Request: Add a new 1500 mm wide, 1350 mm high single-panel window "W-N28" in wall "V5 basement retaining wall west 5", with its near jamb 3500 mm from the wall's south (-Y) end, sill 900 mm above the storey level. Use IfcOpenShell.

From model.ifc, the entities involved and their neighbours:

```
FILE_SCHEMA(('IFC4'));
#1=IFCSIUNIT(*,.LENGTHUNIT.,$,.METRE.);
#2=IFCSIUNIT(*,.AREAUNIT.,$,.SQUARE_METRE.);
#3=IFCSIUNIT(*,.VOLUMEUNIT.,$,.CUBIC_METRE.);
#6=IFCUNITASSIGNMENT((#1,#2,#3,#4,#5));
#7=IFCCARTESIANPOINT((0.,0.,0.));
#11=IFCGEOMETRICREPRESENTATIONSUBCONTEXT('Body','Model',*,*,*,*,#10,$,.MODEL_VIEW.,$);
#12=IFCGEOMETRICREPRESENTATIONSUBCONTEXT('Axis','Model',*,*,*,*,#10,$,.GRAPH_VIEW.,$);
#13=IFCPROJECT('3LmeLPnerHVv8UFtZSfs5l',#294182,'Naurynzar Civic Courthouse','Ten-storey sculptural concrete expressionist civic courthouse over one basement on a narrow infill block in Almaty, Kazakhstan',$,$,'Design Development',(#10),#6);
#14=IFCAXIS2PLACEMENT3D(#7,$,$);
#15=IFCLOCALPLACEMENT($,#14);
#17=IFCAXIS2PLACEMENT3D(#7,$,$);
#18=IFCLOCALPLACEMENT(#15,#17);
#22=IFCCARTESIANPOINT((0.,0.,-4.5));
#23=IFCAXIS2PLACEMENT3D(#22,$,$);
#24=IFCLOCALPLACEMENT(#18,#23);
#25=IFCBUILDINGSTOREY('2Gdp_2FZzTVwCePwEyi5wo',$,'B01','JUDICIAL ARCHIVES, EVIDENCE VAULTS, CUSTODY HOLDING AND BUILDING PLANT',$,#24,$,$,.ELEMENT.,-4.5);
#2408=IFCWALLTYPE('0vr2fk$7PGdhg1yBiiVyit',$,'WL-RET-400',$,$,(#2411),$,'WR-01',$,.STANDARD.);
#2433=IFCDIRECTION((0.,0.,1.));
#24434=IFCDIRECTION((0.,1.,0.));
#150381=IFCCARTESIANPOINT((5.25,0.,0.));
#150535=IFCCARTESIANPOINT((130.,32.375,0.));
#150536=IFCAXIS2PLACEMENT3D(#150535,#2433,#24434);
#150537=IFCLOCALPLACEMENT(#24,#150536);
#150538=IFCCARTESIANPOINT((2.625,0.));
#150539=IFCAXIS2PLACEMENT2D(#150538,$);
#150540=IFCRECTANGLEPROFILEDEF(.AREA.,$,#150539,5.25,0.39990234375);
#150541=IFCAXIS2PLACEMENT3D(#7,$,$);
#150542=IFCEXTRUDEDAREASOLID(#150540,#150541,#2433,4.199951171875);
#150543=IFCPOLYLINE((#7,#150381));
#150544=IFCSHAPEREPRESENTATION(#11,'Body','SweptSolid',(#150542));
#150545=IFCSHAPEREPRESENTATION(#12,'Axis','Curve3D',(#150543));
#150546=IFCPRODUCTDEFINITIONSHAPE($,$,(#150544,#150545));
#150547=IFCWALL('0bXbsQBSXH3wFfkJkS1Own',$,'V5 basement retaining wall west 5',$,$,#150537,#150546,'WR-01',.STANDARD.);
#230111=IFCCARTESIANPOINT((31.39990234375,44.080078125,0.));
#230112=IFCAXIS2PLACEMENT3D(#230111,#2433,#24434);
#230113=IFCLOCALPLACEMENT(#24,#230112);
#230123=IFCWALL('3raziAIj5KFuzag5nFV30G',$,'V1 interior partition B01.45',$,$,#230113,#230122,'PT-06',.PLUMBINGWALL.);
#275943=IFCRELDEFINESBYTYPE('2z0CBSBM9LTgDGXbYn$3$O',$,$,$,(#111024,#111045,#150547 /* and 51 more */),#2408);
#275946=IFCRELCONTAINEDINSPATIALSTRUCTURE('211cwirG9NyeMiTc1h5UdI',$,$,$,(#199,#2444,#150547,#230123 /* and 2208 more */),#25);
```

```python
import numpy as np
import ifcopenshell
import ifcopenshell.api.feature
import ifcopenshell.api.geometry
import ifcopenshell.api.root
import ifcopenshell.api.spatial
import ifcopenshell.geom
import ifcopenshell.util.element
import ifcopenshell.util.placement
import ifcopenshell.util.representation
import ifcopenshell.util.shape
import ifcopenshell.util.unit

model = ifcopenshell.open("model.ifc")
unit_scale = ifcopenshell.util.unit.calculate_unit_scale(model)
settings = ifcopenshell.geom.settings()


def volume(element):
    """Net volume in cubic metres, openings subtracted."""
    shape = ifcopenshell.geom.create_shape(settings, element)
    return ifcopenshell.util.shape.get_volume(shape.geometry)


wall = model.by_guid("0bXbsQBSXH3wFfkJkS1Own")
storey = ifcopenshell.util.element.get_container(wall, ifc_class="IfcBuildingStorey")
context = ifcopenshell.util.representation.get_context(model, "Model", "Body", "MODEL_VIEW")
before = volume(wall)

width, height, from_end, sill = 1.5, 1.35, 3.5, 0.9  # metres

# The wall runs along its own X axis, and the end named is its -X end.
wall_shape = ifcopenshell.geom.create_shape(settings, wall)
x, y, z = ifcopenshell.util.shape.get_vertices(wall_shape.geometry).T
start = x.min() + from_end
face, thickness = float(y.min()), float(y.max() - y.min())
wall_matrix = ifcopenshell.util.placement.get_local_placement(wall.ObjectPlacement)
level = ifcopenshell.util.placement.get_local_placement(storey.ObjectPlacement)[2, 3]


def in_wall(x, y):
    """Placement at x, y metres in the wall's axes, at sill height."""
    matrix = wall_matrix.copy()
    matrix[:, 3] = wall_matrix @ np.array([x / unit_scale, y / unit_scale, 0.0, 1.0])
    matrix[2, 3] = level + sill / unit_scale
    return matrix


# Opening: a box that overshoots both wall faces by 50 mm.
opening = ifcopenshell.api.root.create_entity(model, ifc_class="IfcOpeningElement", predefined_type="OPENING")
box = ifcopenshell.api.geometry.add_wall_representation(
    model, context=context, length=width, height=height, thickness=thickness + 0.1
)
ifcopenshell.api.geometry.assign_representation(model, product=opening, representation=box)
ifcopenshell.api.geometry.edit_object_placement(model, product=opening, matrix=in_wall(start, face - 0.05), is_si=False)
ifcopenshell.api.feature.add_feature(model, feature=opening, element=wall)

window = ifcopenshell.api.root.create_entity(model, ifc_class="IfcWindow", name="W-N28", predefined_type="WINDOW")
window.OverallWidth, window.OverallHeight = width / unit_scale, height / unit_scale
window.PartitioningType = "SINGLE_PANEL"
body = ifcopenshell.api.geometry.add_window_representation(
    model,
    context=context,
    overall_width=window.OverallWidth,
    overall_height=window.OverallHeight,
    partition_type="SINGLE_PANEL",
)
ifcopenshell.api.geometry.assign_representation(model, product=window, representation=body)
ifcopenshell.api.spatial.assign_container(model, products=[window], relating_structure=storey)
ifcopenshell.api.feature.add_filling(model, opening=opening, element=window)

# Centre the window in the wall's thickness.
ifcopenshell.api.geometry.edit_object_placement(model, product=window, matrix=in_wall(start, face), is_si=False)
window_shape = ifcopenshell.geom.create_shape(settings, window)
depth = ifcopenshell.util.shape.get_vertices(window_shape.geometry)[:, 1]
offset = face + thickness / 2 - (depth.min() + depth.max()) / 2
ifcopenshell.api.geometry.edit_object_placement(model, product=window, matrix=in_wall(start, offset), is_si=False)

after = volume(wall)

print(f"wall volume {before:.3f} -> {after:.3f} m3")

model.write("model_edited.ifc")
```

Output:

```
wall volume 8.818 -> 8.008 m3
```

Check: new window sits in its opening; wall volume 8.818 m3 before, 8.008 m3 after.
